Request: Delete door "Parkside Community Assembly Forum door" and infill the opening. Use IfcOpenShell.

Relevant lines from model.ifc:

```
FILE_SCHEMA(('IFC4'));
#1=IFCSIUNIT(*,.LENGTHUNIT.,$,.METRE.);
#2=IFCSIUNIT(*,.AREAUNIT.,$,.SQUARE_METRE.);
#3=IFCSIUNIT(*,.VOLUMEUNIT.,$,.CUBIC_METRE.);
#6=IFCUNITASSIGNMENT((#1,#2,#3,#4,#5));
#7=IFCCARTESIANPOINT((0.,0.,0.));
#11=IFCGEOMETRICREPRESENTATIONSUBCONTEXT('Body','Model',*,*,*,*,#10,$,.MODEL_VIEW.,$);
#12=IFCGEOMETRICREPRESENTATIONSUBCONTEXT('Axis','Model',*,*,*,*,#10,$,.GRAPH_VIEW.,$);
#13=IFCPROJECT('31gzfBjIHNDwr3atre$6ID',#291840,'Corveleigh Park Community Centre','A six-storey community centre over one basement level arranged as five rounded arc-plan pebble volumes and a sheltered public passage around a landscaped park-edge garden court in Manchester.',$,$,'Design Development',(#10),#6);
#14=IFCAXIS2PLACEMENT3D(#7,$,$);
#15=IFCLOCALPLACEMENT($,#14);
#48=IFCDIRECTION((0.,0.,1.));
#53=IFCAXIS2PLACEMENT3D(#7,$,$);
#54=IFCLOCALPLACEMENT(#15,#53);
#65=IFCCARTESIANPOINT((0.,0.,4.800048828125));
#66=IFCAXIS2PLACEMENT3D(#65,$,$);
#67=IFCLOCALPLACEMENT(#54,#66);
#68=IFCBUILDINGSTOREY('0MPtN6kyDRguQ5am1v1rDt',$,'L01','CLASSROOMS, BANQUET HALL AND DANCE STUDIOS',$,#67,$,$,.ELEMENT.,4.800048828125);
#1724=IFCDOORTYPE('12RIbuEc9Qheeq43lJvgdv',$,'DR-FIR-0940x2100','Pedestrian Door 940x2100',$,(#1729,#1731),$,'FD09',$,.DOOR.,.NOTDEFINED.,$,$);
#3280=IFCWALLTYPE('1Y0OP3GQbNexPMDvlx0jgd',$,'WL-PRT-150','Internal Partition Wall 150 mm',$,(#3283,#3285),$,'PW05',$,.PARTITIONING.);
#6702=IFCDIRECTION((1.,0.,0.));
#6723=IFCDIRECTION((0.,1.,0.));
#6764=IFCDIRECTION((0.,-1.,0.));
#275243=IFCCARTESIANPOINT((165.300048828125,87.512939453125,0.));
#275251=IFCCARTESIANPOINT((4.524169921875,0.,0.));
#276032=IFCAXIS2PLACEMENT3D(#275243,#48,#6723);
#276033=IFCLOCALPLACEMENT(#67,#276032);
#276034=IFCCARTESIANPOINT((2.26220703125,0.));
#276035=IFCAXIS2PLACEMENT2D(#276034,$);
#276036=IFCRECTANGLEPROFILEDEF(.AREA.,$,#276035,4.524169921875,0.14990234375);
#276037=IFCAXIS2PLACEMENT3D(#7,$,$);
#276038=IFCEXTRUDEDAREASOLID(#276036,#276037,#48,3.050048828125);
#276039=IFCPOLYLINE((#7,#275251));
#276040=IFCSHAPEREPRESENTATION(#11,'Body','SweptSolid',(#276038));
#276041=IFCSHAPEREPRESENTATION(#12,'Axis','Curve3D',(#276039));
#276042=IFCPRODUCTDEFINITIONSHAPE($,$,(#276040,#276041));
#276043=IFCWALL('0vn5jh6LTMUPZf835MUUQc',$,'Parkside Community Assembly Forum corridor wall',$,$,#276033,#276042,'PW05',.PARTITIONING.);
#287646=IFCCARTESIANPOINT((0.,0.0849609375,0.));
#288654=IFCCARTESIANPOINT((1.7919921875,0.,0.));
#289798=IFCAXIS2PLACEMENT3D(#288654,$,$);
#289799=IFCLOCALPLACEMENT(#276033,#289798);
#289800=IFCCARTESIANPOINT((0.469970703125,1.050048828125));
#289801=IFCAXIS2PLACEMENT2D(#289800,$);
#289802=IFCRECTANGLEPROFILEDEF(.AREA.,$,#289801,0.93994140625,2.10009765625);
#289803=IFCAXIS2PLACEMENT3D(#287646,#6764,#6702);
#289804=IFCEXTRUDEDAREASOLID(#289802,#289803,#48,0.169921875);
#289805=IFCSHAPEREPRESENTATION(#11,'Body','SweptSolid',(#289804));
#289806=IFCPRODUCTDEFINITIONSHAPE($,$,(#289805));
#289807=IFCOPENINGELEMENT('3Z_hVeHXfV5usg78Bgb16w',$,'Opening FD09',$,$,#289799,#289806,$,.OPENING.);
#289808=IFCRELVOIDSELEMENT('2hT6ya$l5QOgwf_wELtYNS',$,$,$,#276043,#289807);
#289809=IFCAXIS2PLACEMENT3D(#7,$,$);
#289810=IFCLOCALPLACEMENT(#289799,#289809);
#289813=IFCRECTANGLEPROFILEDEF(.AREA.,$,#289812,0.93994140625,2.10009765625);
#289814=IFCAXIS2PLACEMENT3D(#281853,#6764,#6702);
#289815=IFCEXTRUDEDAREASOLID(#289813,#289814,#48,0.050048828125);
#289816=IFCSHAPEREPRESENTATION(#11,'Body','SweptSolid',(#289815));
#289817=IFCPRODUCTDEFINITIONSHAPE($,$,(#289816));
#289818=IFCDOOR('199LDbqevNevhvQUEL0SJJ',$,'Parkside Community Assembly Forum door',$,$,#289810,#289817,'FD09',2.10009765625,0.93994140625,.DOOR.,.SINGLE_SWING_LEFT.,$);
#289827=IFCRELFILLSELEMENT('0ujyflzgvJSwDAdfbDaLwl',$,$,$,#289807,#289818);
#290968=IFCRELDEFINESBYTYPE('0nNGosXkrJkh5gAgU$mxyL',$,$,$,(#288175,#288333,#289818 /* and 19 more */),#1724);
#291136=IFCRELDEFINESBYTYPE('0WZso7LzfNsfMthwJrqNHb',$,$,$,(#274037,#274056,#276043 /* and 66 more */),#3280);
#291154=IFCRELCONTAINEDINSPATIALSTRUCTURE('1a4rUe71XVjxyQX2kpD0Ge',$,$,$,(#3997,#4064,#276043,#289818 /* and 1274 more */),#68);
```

```python
import ifcopenshell
import ifcopenshell.api.feature
import ifcopenshell.api.root
import ifcopenshell.geom
import ifcopenshell.util.shape

model = ifcopenshell.open("model.ifc")
settings = ifcopenshell.geom.settings()


def volume(element):
    """Net volume in cubic metres, openings subtracted."""
    shape = ifcopenshell.geom.create_shape(settings, element)
    return ifcopenshell.util.shape.get_volume(shape.geometry)


door = model.by_id(289818)
opening = door.FillsVoids[0].RelatingOpeningElement
wall = opening.VoidsElements[0].RelatingBuildingElement
before = volume(wall)

ifcopenshell.api.root.remove_product(model, product=door)
ifcopenshell.api.feature.remove_feature(model, feature=opening)

after = volume(wall)

print(f"wall volume {before:.3f} -> {after:.3f} m3")

model.write("model-out.ifc")
```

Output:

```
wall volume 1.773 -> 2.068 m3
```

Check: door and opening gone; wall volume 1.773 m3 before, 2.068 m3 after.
